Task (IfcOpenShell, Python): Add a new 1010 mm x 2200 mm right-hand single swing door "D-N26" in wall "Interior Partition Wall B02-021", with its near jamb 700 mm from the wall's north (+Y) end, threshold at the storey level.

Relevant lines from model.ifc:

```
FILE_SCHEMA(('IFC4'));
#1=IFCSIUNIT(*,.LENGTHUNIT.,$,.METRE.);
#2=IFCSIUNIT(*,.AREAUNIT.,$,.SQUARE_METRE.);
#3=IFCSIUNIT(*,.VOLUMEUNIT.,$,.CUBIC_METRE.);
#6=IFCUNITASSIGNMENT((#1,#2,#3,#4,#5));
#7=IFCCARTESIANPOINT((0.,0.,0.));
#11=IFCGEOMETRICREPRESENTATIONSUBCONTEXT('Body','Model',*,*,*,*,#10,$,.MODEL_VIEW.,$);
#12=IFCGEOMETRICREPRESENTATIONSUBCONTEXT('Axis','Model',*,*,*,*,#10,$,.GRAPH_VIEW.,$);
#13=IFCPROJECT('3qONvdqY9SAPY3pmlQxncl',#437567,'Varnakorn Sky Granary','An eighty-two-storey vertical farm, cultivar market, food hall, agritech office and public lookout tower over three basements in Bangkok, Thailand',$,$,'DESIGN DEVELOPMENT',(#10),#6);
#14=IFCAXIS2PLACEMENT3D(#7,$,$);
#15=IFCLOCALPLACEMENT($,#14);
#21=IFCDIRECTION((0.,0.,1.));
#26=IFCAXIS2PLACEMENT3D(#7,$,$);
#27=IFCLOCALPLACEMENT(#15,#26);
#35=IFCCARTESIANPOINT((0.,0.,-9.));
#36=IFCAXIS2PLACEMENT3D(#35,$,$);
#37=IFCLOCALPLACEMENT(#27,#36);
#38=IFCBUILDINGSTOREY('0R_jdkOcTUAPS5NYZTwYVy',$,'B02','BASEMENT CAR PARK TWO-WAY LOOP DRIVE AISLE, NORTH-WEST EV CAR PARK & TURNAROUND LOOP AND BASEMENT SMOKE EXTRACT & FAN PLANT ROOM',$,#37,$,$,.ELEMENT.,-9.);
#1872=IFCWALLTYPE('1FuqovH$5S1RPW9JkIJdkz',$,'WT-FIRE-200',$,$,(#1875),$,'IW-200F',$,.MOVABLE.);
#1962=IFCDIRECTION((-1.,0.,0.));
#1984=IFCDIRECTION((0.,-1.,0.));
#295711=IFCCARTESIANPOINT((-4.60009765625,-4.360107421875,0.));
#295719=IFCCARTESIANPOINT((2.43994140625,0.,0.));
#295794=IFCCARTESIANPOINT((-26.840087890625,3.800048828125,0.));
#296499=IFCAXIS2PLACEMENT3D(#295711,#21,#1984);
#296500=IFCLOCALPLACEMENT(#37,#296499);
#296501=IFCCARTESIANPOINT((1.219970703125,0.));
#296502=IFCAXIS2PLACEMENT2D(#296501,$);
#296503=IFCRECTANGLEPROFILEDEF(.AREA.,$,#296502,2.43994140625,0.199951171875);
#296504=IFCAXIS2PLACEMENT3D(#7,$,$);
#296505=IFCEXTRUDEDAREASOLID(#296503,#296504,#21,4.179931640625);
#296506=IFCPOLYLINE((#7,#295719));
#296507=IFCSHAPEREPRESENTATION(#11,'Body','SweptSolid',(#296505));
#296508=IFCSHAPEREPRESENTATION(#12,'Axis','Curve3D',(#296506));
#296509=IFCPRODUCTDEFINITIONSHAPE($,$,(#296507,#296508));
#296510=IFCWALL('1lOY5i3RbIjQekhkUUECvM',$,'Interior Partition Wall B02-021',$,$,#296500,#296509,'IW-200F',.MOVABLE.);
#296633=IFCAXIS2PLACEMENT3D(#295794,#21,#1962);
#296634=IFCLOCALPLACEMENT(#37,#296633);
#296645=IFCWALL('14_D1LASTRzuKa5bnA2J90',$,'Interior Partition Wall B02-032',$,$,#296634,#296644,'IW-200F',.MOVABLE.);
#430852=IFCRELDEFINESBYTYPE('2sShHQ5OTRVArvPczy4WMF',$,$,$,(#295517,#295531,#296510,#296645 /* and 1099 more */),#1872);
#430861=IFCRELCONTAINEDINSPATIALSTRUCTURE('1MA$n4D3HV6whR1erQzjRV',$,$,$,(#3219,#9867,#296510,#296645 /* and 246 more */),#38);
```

```python
import numpy as np
import ifcopenshell
import ifcopenshell.api.feature
import ifcopenshell.api.geometry
import ifcopenshell.api.root
import ifcopenshell.api.spatial
import ifcopenshell.geom
import ifcopenshell.util.element
import ifcopenshell.util.placement
import ifcopenshell.util.representation
import ifcopenshell.util.shape
import ifcopenshell.util.unit

model = ifcopenshell.open("model.ifc")
unit_scale = ifcopenshell.util.unit.calculate_unit_scale(model)
settings = ifcopenshell.geom.settings()


def volume(element):
    """Net volume in cubic metres, openings subtracted."""
    shape = ifcopenshell.geom.create_shape(settings, element)
    return ifcopenshell.util.shape.get_volume(shape.geometry)


wall = model.by_id(296510)
storey = ifcopenshell.util.element.get_container(wall, ifc_class="IfcBuildingStorey")
context = ifcopenshell.util.representation.get_context(model, "Model", "Body", "MODEL_VIEW")
before = volume(wall)

width, height, from_end, sill = 1.01, 2.2, 0.7, 0.0  # metres

# The wall runs along its own X axis, and the end named is its -X end.
wall_shape = ifcopenshell.geom.create_shape(settings, wall)
x, y, z = ifcopenshell.util.shape.get_vertices(wall_shape.geometry).T
start = x.min() + from_end
face, thickness = float(y.min()), float(y.max() - y.min())
wall_matrix = ifcopenshell.util.placement.get_local_placement(wall.ObjectPlacement)
level = ifcopenshell.util.placement.get_local_placement(storey.ObjectPlacement)[2, 3]


def in_wall(x, y):
    """Placement at x, y metres in the wall's axes, at sill height."""
    matrix = wall_matrix.copy()
    matrix[:, 3] = wall_matrix @ np.array([x / unit_scale, y / unit_scale, 0.0, 1.0])
    matrix[2, 3] = level + sill / unit_scale
    return matrix


# Opening: a box that overshoots both wall faces by 50 mm.
opening = ifcopenshell.api.root.create_entity(model, ifc_class="IfcOpeningElement", predefined_type="OPENING")
box = ifcopenshell.api.geometry.add_wall_representation(
    model, context=context, length=width, height=height, thickness=thickness + 0.1
)
ifcopenshell.api.geometry.assign_representation(model, product=opening, representation=box)
ifcopenshell.api.geometry.edit_object_placement(model, product=opening, matrix=in_wall(start, face - 0.05), is_si=False)
ifcopenshell.api.feature.add_feature(model, feature=opening, element=wall)

door = ifcopenshell.api.root.create_entity(model, ifc_class="IfcDoor", name="D-N26", predefined_type="DOOR")
door.OverallWidth, door.OverallHeight = width / unit_scale, height / unit_scale
door.OperationType = "SINGLE_SWING_RIGHT"
body = ifcopenshell.api.geometry.add_door_representation(
    model,
    context=context,
    overall_width=door.OverallWidth,
    overall_height=door.OverallHeight,
    operation_type="SINGLE_SWING_RIGHT",
    lining_properties={"LiningDepth": thickness / unit_scale, "ThresholdDepth": thickness / unit_scale},
)
ifcopenshell.api.geometry.assign_representation(model, product=door, representation=body)
ifcopenshell.api.spatial.assign_container(model, products=[door], relating_structure=storey)
ifcopenshell.api.feature.add_filling(model, opening=opening, element=door)

# The lining spans the wall, so the door starts at the wall face.
ifcopenshell.api.geometry.edit_object_placement(model, product=door, matrix=in_wall(start, face), is_si=False)

after = volume(wall)

print(f"wall volume {before:.3f} -> {after:.3f} m3")

model.write("model_updated.ifc")
```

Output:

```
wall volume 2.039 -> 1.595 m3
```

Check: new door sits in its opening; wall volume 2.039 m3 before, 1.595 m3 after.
